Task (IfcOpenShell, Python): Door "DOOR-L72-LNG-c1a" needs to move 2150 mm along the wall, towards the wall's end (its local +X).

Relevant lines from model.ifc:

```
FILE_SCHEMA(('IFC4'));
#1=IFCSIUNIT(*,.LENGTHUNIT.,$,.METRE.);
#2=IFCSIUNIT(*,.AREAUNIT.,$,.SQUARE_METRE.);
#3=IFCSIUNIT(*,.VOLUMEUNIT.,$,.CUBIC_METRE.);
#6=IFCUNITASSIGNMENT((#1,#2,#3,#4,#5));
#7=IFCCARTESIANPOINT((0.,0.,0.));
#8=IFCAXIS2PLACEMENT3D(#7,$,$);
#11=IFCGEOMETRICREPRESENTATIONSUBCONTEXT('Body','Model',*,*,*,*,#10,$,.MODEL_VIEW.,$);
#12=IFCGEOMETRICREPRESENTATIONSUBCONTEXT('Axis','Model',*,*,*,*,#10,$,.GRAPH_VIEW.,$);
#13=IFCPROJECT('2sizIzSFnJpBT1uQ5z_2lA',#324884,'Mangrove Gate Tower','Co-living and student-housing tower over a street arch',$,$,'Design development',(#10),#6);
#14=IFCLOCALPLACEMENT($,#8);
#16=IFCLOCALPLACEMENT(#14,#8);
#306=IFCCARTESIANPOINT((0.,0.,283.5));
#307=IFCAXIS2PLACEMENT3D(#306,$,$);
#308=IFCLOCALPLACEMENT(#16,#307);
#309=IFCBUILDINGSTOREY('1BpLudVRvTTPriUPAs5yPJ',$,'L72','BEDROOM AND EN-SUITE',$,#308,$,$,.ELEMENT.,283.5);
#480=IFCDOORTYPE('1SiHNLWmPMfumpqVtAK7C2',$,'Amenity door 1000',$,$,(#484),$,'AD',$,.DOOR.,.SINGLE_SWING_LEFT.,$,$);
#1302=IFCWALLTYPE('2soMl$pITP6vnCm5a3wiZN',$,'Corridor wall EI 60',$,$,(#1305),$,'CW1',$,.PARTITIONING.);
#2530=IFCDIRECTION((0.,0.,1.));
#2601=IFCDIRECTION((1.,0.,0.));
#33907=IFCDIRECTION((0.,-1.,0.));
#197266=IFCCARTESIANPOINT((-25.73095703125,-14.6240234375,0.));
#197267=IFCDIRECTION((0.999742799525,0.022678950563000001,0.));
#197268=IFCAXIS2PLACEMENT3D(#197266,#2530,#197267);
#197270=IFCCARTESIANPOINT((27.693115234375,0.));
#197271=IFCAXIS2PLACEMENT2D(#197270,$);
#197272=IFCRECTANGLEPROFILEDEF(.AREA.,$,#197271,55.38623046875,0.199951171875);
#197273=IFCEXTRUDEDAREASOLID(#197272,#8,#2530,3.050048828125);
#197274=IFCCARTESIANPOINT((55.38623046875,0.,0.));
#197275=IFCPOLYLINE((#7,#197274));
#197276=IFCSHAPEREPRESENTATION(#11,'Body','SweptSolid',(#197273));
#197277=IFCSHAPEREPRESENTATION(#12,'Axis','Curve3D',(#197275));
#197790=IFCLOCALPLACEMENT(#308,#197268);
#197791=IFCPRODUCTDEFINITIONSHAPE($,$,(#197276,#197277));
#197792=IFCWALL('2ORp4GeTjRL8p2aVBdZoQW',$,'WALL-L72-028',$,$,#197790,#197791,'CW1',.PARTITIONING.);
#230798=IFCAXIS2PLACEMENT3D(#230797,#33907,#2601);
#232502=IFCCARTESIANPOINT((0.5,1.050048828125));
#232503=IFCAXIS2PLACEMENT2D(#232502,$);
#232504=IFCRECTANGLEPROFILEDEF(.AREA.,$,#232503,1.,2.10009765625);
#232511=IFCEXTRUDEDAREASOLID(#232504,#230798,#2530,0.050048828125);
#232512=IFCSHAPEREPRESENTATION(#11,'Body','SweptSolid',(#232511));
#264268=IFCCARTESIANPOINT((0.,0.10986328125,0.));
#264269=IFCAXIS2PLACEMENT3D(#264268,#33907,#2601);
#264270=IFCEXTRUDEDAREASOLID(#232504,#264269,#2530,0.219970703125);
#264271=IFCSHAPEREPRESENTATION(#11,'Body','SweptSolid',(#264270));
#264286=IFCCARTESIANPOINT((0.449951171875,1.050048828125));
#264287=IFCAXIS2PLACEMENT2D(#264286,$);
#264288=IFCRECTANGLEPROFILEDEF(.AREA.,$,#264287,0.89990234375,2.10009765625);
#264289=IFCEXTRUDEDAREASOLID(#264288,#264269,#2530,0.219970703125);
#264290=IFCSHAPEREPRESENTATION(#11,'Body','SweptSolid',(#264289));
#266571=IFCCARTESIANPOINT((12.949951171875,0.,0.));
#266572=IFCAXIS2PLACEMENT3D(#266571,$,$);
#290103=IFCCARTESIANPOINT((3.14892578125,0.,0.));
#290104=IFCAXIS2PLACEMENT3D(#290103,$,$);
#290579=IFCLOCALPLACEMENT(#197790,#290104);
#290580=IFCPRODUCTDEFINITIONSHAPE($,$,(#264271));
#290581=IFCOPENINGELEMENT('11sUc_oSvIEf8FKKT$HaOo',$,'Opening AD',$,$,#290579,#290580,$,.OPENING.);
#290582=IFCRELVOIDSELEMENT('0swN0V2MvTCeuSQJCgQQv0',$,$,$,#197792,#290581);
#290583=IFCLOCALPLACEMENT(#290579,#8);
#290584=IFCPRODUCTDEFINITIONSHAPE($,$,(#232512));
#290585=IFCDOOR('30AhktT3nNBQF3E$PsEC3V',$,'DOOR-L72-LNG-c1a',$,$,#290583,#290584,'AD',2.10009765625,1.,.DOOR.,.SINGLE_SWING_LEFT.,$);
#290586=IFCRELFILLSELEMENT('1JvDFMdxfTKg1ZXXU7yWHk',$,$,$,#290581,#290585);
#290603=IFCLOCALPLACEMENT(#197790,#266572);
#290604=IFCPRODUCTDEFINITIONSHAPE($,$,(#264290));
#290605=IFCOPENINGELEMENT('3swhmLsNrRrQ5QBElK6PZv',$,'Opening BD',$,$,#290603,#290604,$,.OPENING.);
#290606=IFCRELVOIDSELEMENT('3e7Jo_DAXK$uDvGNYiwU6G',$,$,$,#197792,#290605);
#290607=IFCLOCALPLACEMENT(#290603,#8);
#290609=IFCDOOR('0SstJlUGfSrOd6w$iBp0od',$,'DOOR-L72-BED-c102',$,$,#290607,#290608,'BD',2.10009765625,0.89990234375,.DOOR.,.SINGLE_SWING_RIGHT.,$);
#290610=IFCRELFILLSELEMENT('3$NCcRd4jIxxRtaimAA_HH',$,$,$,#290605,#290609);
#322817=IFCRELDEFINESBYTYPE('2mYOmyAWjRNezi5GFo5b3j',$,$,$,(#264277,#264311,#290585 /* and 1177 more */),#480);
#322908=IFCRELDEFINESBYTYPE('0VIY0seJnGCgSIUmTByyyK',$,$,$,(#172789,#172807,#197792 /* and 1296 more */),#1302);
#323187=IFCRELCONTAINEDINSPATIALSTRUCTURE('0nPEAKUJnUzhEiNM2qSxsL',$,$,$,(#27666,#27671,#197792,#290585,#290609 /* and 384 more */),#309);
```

```python
import ifcopenshell
import ifcopenshell.api.geometry
import ifcopenshell.util.placement

model = ifcopenshell.open("model.ifc")

door = model.by_guid("30AhktT3nNBQF3E$PsEC3V")
opening = door.FillsVoids[0].RelatingOpeningElement
wall = opening.VoidsElements[0].RelatingBuildingElement

wall_matrix = ifcopenshell.util.placement.get_local_placement(wall.ObjectPlacement)
shift = wall_matrix[:3, 0] * 2.15
before = ifcopenshell.util.placement.get_local_placement(door.ObjectPlacement)[:3, 3].copy()

# The door is placed relative to its opening, so it follows when the opening moves.
matrix = ifcopenshell.util.placement.get_local_placement(opening.ObjectPlacement)
matrix[:3, 3] += shift
ifcopenshell.api.geometry.edit_object_placement(
    model, product=opening, matrix=matrix, is_si=False, should_transform_children=True
)

after = ifcopenshell.util.placement.get_local_placement(door.ObjectPlacement)[:3, 3]
print("door moved by", (after - before).round(3) + 0.0)

model.write("model_v2.ifc")
```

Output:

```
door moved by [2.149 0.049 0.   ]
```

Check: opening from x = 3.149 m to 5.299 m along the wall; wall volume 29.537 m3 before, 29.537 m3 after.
